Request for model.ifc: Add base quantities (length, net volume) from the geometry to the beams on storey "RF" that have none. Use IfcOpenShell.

First a look at what the model holds.

```python
import ifcopenshell
import ifcopenshell.util.element
import ifcopenshell.util.unit

model = ifcopenshell.open("model.ifc")
print(model.schema)
for unit_type in ("LENGTHUNIT", "AREAUNIT", "VOLUMEUNIT"):
    print(unit_type, ifcopenshell.util.unit.calculate_unit_scale(model, unit_type))
storey = next(s for s in model.by_type("IfcBuildingStorey") if s.Name == "RF")
beams = [e for e in ifcopenshell.util.element.get_decomposition(storey) if e.is_a("IfcBeam")]
for e in sorted(beams, key=lambda e: e.id()):
    print(e.id(), e.is_a(), e.Name, list(ifcopenshell.util.element.get_psets(e, qtos_only=True)), sep=" | ")
```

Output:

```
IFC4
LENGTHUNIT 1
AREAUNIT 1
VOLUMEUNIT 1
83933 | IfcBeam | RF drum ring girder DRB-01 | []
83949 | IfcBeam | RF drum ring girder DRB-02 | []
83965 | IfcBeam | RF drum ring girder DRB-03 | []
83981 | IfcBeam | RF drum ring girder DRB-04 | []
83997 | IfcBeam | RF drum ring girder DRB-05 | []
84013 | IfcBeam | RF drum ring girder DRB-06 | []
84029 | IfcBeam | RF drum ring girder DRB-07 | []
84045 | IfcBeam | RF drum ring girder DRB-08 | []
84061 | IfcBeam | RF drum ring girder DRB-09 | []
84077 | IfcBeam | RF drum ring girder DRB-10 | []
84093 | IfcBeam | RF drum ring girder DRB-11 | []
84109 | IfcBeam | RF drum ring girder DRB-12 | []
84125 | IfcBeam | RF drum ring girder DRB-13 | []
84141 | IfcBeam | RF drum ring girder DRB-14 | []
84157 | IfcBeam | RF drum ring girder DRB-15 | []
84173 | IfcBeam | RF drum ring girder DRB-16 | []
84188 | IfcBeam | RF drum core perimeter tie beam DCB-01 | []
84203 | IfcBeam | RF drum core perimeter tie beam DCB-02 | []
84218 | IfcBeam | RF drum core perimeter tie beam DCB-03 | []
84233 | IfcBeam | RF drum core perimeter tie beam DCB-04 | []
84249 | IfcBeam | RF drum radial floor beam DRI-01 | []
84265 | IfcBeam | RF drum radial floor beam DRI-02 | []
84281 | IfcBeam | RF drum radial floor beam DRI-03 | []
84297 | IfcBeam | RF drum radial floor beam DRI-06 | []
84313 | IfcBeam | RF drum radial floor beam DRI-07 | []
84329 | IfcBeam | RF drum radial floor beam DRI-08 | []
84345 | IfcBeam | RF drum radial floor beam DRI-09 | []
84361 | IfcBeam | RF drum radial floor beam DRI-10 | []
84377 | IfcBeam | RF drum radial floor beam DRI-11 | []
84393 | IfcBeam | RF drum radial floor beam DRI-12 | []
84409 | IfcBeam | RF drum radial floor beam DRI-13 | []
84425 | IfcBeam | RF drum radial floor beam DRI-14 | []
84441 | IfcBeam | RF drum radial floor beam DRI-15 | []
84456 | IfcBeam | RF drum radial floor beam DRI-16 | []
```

```python
import ifcopenshell
import ifcopenshell.api.pset
import ifcopenshell.geom
import ifcopenshell.util.element
import ifcopenshell.util.shape
import ifcopenshell.util.unit

model = ifcopenshell.open("model.ifc")
unit_scale = ifcopenshell.util.unit.calculate_unit_scale(model)
volume_scale = ifcopenshell.util.unit.calculate_unit_scale(model, "VOLUMEUNIT")
settings = ifcopenshell.geom.settings()

storey = next(s for s in model.by_type("IfcBuildingStorey") if s.Name == "RF")
beams = [e for e in ifcopenshell.util.element.get_decomposition(storey) if e.is_a("IfcBeam")]

for e in sorted(beams, key=lambda e: e.id()):
    if ifcopenshell.util.element.get_psets(e, qtos_only=True, should_inherit=False):
        continue
    # Geometry comes back in metres, in the element's own axes.
    shape = ifcopenshell.geom.create_shape(settings, e)
    values = {
        "Length": ifcopenshell.util.shape.get_max_xyz(shape.geometry) / unit_scale,
        "NetVolume": ifcopenshell.util.shape.get_volume(shape.geometry) / volume_scale,
    }
    qto = ifcopenshell.api.pset.add_qto(model, product=e, name="Qto_BeamBaseQuantities")
    ifcopenshell.api.pset.edit_qto(model, qto=qto, properties=values)
    print(e.id(), {k: round(v, 3) for k, v in values.items()})

model.write("model_rev.ifc")
```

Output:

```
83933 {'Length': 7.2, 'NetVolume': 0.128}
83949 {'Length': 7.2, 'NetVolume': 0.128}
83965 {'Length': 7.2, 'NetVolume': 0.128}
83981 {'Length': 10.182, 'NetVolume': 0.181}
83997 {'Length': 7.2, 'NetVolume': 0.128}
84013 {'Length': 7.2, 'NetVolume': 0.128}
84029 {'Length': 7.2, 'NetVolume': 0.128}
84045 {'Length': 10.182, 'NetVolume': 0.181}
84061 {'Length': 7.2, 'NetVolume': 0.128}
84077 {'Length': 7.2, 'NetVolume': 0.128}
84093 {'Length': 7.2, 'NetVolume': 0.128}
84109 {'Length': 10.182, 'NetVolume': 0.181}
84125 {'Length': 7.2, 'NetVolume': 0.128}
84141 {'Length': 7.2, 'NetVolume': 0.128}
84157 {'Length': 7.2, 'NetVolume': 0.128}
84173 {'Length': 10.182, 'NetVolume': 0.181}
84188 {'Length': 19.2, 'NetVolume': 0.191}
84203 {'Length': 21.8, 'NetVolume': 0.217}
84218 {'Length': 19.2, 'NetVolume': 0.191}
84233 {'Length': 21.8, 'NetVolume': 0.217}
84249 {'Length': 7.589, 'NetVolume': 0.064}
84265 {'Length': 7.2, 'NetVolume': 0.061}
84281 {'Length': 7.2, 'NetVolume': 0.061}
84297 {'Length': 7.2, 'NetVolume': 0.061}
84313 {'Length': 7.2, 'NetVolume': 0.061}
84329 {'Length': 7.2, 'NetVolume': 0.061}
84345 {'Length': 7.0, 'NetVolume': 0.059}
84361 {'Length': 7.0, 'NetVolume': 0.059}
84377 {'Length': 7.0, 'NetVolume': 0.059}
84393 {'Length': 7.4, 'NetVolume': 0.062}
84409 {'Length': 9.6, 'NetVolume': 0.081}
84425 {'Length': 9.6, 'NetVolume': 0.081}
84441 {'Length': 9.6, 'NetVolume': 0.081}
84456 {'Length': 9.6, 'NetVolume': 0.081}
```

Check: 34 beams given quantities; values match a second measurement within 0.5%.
